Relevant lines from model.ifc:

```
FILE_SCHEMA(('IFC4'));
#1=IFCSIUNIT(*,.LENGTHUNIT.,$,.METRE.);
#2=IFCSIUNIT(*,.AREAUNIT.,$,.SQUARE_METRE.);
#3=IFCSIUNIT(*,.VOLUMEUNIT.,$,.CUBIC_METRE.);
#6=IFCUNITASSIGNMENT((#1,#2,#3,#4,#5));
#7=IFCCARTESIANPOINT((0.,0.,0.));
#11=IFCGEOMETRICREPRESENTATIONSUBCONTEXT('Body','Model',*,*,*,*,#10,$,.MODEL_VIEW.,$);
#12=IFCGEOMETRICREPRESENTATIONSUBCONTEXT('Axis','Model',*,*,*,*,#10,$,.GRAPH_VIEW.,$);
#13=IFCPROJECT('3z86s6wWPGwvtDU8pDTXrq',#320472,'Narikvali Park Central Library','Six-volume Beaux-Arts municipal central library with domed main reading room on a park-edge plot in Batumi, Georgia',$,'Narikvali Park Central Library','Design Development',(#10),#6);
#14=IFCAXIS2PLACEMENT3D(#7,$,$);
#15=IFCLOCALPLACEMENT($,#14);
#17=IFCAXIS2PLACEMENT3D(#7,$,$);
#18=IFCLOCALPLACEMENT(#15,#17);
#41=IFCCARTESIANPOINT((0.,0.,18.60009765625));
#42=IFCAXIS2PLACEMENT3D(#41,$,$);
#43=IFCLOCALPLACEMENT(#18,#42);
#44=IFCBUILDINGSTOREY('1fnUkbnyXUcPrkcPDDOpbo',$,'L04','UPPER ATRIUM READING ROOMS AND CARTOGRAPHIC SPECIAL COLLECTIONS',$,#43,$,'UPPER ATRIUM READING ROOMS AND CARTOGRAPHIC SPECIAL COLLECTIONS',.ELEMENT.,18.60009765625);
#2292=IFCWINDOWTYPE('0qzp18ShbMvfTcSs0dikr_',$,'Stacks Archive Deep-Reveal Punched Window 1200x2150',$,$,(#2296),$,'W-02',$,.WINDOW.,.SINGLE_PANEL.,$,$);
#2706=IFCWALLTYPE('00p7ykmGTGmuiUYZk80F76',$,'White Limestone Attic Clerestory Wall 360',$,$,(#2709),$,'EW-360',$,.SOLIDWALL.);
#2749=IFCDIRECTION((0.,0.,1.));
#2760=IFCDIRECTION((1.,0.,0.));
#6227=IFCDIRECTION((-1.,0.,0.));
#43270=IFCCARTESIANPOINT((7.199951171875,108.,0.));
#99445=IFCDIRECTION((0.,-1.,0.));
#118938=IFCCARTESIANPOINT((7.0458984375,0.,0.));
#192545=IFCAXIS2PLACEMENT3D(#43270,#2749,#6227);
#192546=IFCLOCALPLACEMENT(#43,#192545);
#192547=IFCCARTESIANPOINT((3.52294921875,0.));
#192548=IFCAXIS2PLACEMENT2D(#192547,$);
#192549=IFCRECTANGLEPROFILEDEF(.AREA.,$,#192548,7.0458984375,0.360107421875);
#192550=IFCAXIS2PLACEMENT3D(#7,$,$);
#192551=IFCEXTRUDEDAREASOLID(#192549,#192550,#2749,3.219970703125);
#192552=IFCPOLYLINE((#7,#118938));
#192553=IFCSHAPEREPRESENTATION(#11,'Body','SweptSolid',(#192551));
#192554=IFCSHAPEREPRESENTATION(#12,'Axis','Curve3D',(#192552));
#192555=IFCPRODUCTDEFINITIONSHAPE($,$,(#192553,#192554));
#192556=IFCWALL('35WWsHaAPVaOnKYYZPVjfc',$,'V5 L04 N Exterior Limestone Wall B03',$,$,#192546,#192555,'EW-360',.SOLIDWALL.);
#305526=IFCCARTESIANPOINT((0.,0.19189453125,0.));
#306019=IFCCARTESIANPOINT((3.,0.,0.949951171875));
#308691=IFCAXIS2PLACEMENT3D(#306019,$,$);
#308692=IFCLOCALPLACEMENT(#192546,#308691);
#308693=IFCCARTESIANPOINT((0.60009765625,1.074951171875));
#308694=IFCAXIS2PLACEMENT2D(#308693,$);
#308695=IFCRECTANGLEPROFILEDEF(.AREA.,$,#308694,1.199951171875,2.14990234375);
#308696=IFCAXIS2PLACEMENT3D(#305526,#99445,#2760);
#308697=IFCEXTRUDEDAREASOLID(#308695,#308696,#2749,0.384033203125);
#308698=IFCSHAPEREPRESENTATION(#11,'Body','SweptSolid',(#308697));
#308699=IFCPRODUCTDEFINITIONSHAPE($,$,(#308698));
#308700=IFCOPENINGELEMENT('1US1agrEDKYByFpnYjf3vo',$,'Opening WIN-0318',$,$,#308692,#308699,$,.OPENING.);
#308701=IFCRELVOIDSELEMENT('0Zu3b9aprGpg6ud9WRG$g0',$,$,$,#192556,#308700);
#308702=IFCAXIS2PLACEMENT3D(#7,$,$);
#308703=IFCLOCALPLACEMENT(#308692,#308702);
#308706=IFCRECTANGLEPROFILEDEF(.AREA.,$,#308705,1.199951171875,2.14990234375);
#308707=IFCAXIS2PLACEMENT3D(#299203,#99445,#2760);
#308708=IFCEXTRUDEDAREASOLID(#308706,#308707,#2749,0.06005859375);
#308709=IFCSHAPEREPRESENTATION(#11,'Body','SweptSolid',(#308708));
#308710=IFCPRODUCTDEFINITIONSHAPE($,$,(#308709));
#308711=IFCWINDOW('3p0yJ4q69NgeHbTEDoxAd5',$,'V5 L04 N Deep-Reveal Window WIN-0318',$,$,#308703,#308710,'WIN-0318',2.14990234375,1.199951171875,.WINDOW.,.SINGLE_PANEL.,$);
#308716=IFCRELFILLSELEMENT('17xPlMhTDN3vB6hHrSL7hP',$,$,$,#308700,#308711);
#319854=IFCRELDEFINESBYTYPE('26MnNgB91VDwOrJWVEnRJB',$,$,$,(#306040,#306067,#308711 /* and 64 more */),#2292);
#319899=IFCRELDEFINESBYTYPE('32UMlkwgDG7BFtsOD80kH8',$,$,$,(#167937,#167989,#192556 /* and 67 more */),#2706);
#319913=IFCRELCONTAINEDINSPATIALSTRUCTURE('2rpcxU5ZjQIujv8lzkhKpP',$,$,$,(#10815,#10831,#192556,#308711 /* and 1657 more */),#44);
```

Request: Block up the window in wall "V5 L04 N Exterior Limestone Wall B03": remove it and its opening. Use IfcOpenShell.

```python
import ifcopenshell
import ifcopenshell.api.feature
import ifcopenshell.api.root
import ifcopenshell.geom
import ifcopenshell.util.shape

model = ifcopenshell.open("model.ifc")
settings = ifcopenshell.geom.settings()


def volume(element):
    """Net volume in cubic metres, openings subtracted."""
    shape = ifcopenshell.geom.create_shape(settings, element)
    return ifcopenshell.util.shape.get_volume(shape.geometry)


window = model.by_id(308711)
opening = window.FillsVoids[0].RelatingOpeningElement
wall = opening.VoidsElements[0].RelatingBuildingElement
before = volume(wall)

ifcopenshell.api.root.remove_product(model, product=window)
ifcopenshell.api.feature.remove_feature(model, feature=opening)

after = volume(wall)

print(f"wall volume {before:.3f} -> {after:.3f} m3")

model.write("model_rev.ifc")
```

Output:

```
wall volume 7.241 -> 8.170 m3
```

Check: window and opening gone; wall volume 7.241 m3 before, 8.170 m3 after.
